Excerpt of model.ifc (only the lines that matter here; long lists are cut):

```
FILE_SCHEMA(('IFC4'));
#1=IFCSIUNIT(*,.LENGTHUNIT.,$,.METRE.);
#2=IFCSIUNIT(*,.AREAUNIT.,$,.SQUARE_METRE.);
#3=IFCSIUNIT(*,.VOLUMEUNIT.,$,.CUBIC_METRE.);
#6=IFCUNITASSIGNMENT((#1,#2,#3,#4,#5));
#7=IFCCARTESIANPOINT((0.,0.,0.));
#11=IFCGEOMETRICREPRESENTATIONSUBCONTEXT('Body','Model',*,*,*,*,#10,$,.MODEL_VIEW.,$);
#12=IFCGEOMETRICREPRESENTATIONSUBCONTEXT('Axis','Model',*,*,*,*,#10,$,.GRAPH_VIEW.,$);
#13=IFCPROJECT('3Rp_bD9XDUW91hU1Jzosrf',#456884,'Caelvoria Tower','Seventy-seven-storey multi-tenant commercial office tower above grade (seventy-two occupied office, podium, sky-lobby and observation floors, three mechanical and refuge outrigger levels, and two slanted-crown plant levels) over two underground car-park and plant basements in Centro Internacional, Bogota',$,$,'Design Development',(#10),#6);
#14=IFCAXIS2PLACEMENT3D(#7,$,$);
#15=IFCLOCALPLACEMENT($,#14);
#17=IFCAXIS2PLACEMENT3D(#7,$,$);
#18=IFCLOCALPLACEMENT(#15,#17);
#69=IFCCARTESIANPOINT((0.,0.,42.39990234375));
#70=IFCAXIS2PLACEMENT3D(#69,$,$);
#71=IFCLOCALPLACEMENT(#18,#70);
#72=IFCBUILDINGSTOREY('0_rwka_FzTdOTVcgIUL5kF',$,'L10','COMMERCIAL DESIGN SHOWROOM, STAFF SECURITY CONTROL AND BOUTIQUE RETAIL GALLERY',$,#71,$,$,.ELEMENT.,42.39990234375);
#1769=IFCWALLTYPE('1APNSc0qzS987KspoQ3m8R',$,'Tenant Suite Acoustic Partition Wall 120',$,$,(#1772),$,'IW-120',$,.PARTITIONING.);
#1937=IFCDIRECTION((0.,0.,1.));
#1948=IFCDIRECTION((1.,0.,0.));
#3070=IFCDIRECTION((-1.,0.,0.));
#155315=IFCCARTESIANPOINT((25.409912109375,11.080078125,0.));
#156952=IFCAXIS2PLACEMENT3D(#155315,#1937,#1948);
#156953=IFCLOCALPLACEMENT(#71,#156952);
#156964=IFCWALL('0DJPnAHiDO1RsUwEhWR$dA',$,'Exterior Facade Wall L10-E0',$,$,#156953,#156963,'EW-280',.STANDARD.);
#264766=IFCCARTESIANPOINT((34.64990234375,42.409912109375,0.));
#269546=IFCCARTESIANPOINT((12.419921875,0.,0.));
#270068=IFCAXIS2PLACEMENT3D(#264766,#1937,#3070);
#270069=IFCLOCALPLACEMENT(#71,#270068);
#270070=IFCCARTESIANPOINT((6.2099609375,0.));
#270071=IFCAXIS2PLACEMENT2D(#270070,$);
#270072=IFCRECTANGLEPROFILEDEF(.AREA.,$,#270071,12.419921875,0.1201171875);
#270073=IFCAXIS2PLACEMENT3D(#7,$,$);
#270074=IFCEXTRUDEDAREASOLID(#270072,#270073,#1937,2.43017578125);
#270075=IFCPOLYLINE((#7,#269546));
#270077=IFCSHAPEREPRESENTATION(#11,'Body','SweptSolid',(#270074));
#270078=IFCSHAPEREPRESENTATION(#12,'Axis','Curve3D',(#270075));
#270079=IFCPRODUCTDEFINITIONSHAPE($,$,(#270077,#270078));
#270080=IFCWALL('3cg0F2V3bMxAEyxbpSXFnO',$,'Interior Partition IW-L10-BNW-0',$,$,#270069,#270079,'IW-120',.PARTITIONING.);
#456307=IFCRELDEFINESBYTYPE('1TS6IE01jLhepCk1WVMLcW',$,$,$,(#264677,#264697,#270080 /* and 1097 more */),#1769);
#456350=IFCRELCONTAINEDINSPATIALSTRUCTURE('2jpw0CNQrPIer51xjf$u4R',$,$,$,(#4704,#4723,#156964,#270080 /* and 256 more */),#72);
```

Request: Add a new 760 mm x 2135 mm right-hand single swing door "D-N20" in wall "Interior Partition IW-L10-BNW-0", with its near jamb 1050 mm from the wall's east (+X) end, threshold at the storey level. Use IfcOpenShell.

```python
import numpy as np
import ifcopenshell
import ifcopenshell.api.feature
import ifcopenshell.api.geometry
import ifcopenshell.api.root
import ifcopenshell.api.spatial
import ifcopenshell.geom
import ifcopenshell.util.element
import ifcopenshell.util.placement
import ifcopenshell.util.representation
import ifcopenshell.util.shape
import ifcopenshell.util.unit

model = ifcopenshell.open("model.ifc")
unit_scale = ifcopenshell.util.unit.calculate_unit_scale(model)
settings = ifcopenshell.geom.settings()


def volume(element):
    """Net volume in cubic metres, openings subtracted."""
    shape = ifcopenshell.geom.create_shape(settings, element)
    return ifcopenshell.util.shape.get_volume(shape.geometry)


wall = model.by_guid("3cg0F2V3bMxAEyxbpSXFnO")
storey = ifcopenshell.util.element.get_container(wall, ifc_class="IfcBuildingStorey")
context = ifcopenshell.util.representation.get_context(model, "Model", "Body", "MODEL_VIEW")
before = volume(wall)

width, height, from_end, sill = 0.76, 2.135, 1.05, 0.0  # metres

# The wall runs along its own X axis, and the end named is its -X end.
wall_shape = ifcopenshell.geom.create_shape(settings, wall)
x, y, z = ifcopenshell.util.shape.get_vertices(wall_shape.geometry).T
start = x.min() + from_end
face, thickness = float(y.min()), float(y.max() - y.min())
wall_matrix = ifcopenshell.util.placement.get_local_placement(wall.ObjectPlacement)
level = ifcopenshell.util.placement.get_local_placement(storey.ObjectPlacement)[2, 3]


def in_wall(x, y):
    """Placement at x, y metres in the wall's axes, at sill height."""
    matrix = wall_matrix.copy()
    matrix[:, 3] = wall_matrix @ np.array([x / unit_scale, y / unit_scale, 0.0, 1.0])
    matrix[2, 3] = level + sill / unit_scale
    return matrix


# Opening: a box that overshoots both wall faces by 50 mm.
opening = ifcopenshell.api.root.create_entity(model, ifc_class="IfcOpeningElement", predefined_type="OPENING")
box = ifcopenshell.api.geometry.add_wall_representation(
    model, context=context, length=width, height=height, thickness=thickness + 0.1
)
ifcopenshell.api.geometry.assign_representation(model, product=opening, representation=box)
ifcopenshell.api.geometry.edit_object_placement(model, product=opening, matrix=in_wall(start, face - 0.05), is_si=False)
ifcopenshell.api.feature.add_feature(model, feature=opening, element=wall)

door = ifcopenshell.api.root.create_entity(model, ifc_class="IfcDoor", name="D-N20", predefined_type="DOOR")
door.OverallWidth, door.OverallHeight = width / unit_scale, height / unit_scale
door.OperationType = "SINGLE_SWING_RIGHT"
body = ifcopenshell.api.geometry.add_door_representation(
    model,
    context=context,
    overall_width=door.OverallWidth,
    overall_height=door.OverallHeight,
    operation_type="SINGLE_SWING_RIGHT",
    lining_properties={"LiningDepth": thickness / unit_scale, "ThresholdDepth": thickness / unit_scale},
)
ifcopenshell.api.geometry.assign_representation(model, product=door, representation=body)
ifcopenshell.api.spatial.assign_container(model, products=[door], relating_structure=storey)
ifcopenshell.api.feature.add_filling(model, opening=opening, element=door)

# The lining spans the wall, so the door starts at the wall face.
ifcopenshell.api.geometry.edit_object_placement(model, product=door, matrix=in_wall(start, face), is_si=False)

after = volume(wall)

print(f"wall volume {before:.3f} -> {after:.3f} m3")

model.write("model_rev.ifc")
```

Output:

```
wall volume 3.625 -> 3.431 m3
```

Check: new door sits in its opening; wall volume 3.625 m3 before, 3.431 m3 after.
